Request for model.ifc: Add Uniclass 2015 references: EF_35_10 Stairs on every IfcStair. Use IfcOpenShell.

First a look at what the model holds.

```python
import ifcopenshell

model = ifcopenshell.open("model.ifc")
print(model.schema)
print("classifications:", [c.Name for c in model.by_type("IfcClassification")])
for ifc_class in ("IfcDoor", "IfcRoof", "IfcStair", "IfcWall", "IfcWindow"):
    print(ifc_class, len(model.by_type(ifc_class)))
```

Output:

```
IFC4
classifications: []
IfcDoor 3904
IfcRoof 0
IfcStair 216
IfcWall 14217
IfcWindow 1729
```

```python
import ifcopenshell
import ifcopenshell.api.classification

model = ifcopenshell.open("model.ifc")

system = ifcopenshell.api.classification.add_classification(model, classification="Uniclass 2015")

codes = {
    "IfcStair": ("EF_35_10", "Stairs"),
}
for ifc_class, (code, name) in codes.items():
    products = model.by_type(ifc_class)
    ifcopenshell.api.classification.add_reference(
        model, products=products, classification=system, identification=code, name=name
    )
    print(code, len(products))

model.write("model_rev.ifc")
```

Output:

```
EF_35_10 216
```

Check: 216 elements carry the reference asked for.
